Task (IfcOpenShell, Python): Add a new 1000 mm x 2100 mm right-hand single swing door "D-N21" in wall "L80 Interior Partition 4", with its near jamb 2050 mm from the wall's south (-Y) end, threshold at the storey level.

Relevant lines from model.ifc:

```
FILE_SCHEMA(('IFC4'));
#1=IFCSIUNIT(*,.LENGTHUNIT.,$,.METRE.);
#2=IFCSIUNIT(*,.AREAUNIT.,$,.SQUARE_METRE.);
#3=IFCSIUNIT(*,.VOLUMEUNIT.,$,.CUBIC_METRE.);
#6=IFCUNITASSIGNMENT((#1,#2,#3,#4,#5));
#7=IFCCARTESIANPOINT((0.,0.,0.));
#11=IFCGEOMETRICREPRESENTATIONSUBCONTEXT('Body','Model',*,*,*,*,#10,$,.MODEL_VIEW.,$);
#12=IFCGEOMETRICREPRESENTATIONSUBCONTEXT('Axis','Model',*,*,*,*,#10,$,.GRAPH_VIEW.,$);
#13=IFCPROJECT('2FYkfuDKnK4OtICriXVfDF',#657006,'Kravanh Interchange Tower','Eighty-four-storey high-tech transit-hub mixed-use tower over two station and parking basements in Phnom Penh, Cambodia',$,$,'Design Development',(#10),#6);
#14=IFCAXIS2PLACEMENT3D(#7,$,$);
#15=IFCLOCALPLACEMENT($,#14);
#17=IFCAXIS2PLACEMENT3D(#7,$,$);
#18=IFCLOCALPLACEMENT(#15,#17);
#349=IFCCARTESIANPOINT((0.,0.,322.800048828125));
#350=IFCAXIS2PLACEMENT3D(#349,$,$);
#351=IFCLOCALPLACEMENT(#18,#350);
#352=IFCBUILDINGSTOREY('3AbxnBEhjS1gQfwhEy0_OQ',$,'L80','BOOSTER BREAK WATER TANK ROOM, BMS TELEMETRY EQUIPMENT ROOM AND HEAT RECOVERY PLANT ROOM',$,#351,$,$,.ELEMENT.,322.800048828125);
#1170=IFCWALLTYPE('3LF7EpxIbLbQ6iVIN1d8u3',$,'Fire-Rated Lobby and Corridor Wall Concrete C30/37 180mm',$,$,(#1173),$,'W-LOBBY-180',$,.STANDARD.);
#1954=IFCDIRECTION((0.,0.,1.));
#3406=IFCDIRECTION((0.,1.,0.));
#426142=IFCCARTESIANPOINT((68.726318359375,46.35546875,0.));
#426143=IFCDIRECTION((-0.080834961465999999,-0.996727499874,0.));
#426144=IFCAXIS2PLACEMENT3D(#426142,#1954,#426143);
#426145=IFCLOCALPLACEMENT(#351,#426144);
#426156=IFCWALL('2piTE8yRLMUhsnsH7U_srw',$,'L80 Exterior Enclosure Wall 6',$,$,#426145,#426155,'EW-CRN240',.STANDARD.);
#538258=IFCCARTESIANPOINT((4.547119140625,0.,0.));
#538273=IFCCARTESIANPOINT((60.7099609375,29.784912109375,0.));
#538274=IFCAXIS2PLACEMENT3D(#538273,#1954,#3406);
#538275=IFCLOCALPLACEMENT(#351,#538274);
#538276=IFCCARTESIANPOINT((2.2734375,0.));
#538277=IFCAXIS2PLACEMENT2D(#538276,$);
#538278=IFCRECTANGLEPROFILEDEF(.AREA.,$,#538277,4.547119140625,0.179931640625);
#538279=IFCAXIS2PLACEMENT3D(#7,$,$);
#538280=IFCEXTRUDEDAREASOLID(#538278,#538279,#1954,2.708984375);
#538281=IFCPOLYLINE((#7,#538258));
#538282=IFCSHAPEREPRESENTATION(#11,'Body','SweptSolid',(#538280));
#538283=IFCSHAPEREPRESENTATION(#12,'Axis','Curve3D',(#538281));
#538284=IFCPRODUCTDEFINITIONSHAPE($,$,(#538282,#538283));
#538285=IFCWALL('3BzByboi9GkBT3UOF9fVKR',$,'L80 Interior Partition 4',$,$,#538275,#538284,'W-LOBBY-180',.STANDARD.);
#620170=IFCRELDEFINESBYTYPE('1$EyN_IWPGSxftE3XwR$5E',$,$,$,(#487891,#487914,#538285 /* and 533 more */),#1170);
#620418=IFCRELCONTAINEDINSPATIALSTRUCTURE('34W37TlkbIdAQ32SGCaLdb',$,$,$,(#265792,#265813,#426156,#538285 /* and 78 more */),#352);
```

```python
import numpy as np
import ifcopenshell
import ifcopenshell.api.feature
import ifcopenshell.api.geometry
import ifcopenshell.api.root
import ifcopenshell.api.spatial
import ifcopenshell.geom
import ifcopenshell.util.element
import ifcopenshell.util.placement
import ifcopenshell.util.representation
import ifcopenshell.util.shape
import ifcopenshell.util.unit

model = ifcopenshell.open("model.ifc")
unit_scale = ifcopenshell.util.unit.calculate_unit_scale(model)
settings = ifcopenshell.geom.settings()


def volume(element):
    """Net volume in cubic metres, openings subtracted."""
    shape = ifcopenshell.geom.create_shape(settings, element)
    return ifcopenshell.util.shape.get_volume(shape.geometry)


wall = model.by_guid("3BzByboi9GkBT3UOF9fVKR")
storey = ifcopenshell.util.element.get_container(wall, ifc_class="IfcBuildingStorey")
context = ifcopenshell.util.representation.get_context(model, "Model", "Body", "MODEL_VIEW")
before = volume(wall)

width, height, from_end, sill = 1, 2.1, 2.05, 0.0  # metres

# The wall runs along its own X axis, and the end named is its -X end.
wall_shape = ifcopenshell.geom.create_shape(settings, wall)
x, y, z = ifcopenshell.util.shape.get_vertices(wall_shape.geometry).T
start = x.min() + from_end
face, thickness = float(y.min()), float(y.max() - y.min())
wall_matrix = ifcopenshell.util.placement.get_local_placement(wall.ObjectPlacement)
level = ifcopenshell.util.placement.get_local_placement(storey.ObjectPlacement)[2, 3]


def in_wall(x, y):
    """Placement at x, y metres in the wall's axes, at sill height."""
    matrix = wall_matrix.copy()
    matrix[:, 3] = wall_matrix @ np.array([x / unit_scale, y / unit_scale, 0.0, 1.0])
    matrix[2, 3] = level + sill / unit_scale
    return matrix


# Opening: a box that overshoots both wall faces by 50 mm.
opening = ifcopenshell.api.root.create_entity(model, ifc_class="IfcOpeningElement", predefined_type="OPENING")
box = ifcopenshell.api.geometry.add_wall_representation(
    model, context=context, length=width, height=height, thickness=thickness + 0.1
)
ifcopenshell.api.geometry.assign_representation(model, product=opening, representation=box)
ifcopenshell.api.geometry.edit_object_placement(model, product=opening, matrix=in_wall(start, face - 0.05), is_si=False)
ifcopenshell.api.feature.add_feature(model, feature=opening, element=wall)

door = ifcopenshell.api.root.create_entity(model, ifc_class="IfcDoor", name="D-N21", predefined_type="DOOR")
door.OverallWidth, door.OverallHeight = width / unit_scale, height / unit_scale
door.OperationType = "SINGLE_SWING_RIGHT"
body = ifcopenshell.api.geometry.add_door_representation(
    model,
    context=context,
    overall_width=door.OverallWidth,
    overall_height=door.OverallHeight,
    operation_type="SINGLE_SWING_RIGHT",
    lining_properties={"LiningDepth": thickness / unit_scale, "ThresholdDepth": thickness / unit_scale},
)
ifcopenshell.api.geometry.assign_representation(model, product=door, representation=body)
ifcopenshell.api.spatial.assign_container(model, products=[door], relating_structure=storey)
ifcopenshell.api.feature.add_filling(model, opening=opening, element=door)

# The lining spans the wall, so the door starts at the wall face.
ifcopenshell.api.geometry.edit_object_placement(model, product=door, matrix=in_wall(start, face), is_si=False)

after = volume(wall)

print(f"wall volume {before:.3f} -> {after:.3f} m3")

model.write("model-out.ifc")
```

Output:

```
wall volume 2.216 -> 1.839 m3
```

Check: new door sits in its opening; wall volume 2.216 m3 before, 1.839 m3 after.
